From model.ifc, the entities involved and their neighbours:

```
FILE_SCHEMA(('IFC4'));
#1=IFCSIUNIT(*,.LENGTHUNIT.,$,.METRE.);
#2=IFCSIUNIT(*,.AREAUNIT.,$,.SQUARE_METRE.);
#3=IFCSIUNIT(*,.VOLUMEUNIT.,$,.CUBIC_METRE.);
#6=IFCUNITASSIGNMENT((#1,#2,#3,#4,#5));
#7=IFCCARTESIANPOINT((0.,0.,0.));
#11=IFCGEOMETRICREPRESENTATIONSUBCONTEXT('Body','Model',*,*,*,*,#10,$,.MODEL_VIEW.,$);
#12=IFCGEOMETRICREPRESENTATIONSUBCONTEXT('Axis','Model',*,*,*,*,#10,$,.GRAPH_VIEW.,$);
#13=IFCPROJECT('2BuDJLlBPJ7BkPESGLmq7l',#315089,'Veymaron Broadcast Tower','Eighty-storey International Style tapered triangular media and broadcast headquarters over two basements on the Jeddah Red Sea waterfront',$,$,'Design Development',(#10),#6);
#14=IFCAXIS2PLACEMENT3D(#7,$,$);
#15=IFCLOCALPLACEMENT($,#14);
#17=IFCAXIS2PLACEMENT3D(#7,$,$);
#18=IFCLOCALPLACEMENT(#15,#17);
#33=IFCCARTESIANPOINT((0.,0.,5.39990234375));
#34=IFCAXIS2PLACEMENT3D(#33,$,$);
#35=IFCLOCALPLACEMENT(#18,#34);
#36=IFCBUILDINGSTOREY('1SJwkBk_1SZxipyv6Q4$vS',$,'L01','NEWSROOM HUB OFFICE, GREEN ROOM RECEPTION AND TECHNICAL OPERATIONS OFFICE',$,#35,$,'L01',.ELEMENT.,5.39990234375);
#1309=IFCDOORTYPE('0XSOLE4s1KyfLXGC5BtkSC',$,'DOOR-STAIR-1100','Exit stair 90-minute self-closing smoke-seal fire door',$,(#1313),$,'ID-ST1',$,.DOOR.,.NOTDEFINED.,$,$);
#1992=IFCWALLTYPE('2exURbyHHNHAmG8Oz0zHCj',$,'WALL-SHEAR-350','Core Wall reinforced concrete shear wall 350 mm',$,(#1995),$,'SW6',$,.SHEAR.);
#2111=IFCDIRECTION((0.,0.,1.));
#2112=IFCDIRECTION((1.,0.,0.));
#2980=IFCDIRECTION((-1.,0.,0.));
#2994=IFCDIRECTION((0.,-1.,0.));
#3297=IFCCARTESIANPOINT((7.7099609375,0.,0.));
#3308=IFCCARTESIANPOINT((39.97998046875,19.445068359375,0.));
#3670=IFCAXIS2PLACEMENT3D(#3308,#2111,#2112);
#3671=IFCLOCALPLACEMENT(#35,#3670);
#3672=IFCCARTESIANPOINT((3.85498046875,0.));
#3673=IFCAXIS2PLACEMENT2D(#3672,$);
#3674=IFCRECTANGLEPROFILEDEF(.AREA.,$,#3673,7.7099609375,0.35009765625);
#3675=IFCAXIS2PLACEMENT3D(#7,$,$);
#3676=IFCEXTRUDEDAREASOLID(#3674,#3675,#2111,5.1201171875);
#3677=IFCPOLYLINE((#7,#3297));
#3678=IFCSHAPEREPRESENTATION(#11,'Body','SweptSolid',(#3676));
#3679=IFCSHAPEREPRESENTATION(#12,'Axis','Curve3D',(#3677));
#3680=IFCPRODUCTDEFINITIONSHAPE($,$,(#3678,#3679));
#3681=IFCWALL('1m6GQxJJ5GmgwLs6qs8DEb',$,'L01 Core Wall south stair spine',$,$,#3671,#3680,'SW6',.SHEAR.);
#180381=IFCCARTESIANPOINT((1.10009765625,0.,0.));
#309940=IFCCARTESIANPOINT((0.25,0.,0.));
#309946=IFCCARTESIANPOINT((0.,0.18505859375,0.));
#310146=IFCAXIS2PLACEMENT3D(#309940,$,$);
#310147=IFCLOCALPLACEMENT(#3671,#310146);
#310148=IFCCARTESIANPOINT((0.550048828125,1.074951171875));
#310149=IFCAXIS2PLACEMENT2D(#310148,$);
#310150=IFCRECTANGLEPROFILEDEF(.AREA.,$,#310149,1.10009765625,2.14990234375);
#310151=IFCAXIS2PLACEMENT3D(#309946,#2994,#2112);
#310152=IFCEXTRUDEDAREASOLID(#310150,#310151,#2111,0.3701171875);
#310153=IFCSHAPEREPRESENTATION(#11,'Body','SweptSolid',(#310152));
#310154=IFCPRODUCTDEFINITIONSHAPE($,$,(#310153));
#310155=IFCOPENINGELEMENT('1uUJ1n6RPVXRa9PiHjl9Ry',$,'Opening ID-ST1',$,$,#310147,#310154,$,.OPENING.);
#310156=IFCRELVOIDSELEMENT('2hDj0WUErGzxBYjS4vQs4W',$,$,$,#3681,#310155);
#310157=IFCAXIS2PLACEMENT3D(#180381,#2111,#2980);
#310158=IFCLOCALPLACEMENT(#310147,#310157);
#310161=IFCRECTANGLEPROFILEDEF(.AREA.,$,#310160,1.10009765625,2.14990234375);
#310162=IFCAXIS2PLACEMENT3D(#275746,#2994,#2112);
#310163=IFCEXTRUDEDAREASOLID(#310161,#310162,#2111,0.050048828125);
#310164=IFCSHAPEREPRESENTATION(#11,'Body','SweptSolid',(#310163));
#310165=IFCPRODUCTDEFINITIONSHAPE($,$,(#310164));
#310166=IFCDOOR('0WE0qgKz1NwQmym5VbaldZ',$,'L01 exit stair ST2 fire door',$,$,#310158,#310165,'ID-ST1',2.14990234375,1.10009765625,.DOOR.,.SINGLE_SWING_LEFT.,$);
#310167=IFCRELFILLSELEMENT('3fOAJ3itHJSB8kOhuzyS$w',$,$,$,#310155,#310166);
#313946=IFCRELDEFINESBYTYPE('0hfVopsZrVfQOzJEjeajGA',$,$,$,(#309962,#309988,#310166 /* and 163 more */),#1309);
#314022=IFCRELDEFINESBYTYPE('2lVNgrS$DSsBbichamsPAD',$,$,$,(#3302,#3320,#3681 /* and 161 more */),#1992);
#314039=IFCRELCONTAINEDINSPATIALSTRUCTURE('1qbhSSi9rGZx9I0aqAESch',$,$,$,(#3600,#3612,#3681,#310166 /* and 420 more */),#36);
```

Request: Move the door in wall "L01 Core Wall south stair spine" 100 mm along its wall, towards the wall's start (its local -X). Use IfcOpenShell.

```python
import ifcopenshell
import ifcopenshell.api.geometry
import ifcopenshell.util.placement
import ifcopenshell.util.unit

model = ifcopenshell.open("model.ifc")
unit_scale = ifcopenshell.util.unit.calculate_unit_scale(model)

door = model.by_guid("0WE0qgKz1NwQmym5VbaldZ")
opening = door.FillsVoids[0].RelatingOpeningElement
wall = opening.VoidsElements[0].RelatingBuildingElement

wall_matrix = ifcopenshell.util.placement.get_local_placement(wall.ObjectPlacement)
shift = wall_matrix[:3, 0] * -0.1 / unit_scale
before = ifcopenshell.util.placement.get_local_placement(door.ObjectPlacement)[:3, 3].copy()

# The door is placed relative to its opening, so it follows when the opening moves.
matrix = ifcopenshell.util.placement.get_local_placement(opening.ObjectPlacement)
matrix[:3, 3] += shift
ifcopenshell.api.geometry.edit_object_placement(
    model, product=opening, matrix=matrix, is_si=False, should_transform_children=True
)

after = ifcopenshell.util.placement.get_local_placement(door.ObjectPlacement)[:3, 3]
print("door moved by", (after - before).round(3) + 0.0)

model.write("model_updated.ifc")
```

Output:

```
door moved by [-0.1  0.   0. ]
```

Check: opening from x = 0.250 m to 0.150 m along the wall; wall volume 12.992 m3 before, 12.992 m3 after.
